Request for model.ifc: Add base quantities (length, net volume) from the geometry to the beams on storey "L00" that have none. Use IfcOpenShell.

First a look at what the model holds.

```python
import ifcopenshell
import ifcopenshell.util.element
import ifcopenshell.util.unit

model = ifcopenshell.open("model.ifc")
print(model.schema)
for unit_type in ("LENGTHUNIT", "AREAUNIT", "VOLUMEUNIT"):
    print(unit_type, ifcopenshell.util.unit.calculate_unit_scale(model, unit_type))
storey = next(s for s in model.by_type("IfcBuildingStorey") if s.Name == "L00")
beams = [e for e in ifcopenshell.util.element.get_decomposition(storey) if e.is_a("IfcBeam")]
for e in sorted(beams, key=lambda e: e.id()):
    print(e.id(), e.is_a(), e.Name, list(ifcopenshell.util.element.get_psets(e, qtos_only=True)), sep=" | ")
```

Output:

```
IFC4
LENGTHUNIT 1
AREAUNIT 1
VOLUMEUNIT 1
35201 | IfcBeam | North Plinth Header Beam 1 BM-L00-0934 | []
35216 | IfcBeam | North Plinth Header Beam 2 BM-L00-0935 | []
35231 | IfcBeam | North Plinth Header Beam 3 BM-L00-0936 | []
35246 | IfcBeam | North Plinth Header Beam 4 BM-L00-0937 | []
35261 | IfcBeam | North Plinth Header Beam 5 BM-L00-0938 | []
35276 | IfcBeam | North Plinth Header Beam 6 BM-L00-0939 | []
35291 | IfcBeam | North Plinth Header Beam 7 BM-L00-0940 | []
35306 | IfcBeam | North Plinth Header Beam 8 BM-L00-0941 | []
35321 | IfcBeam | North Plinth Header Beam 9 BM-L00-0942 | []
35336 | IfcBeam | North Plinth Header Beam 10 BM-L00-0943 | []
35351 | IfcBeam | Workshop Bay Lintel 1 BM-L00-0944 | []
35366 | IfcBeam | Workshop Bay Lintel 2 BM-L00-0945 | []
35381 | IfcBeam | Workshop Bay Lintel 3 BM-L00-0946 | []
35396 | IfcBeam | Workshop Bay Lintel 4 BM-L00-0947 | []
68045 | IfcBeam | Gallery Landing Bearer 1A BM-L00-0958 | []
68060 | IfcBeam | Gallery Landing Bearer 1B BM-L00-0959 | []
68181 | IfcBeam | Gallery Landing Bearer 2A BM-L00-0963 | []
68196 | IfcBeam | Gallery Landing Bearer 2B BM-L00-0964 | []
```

```python
import ifcopenshell
import ifcopenshell.api.pset
import ifcopenshell.geom
import ifcopenshell.util.element
import ifcopenshell.util.shape
import ifcopenshell.util.unit

model = ifcopenshell.open("model.ifc")
unit_scale = ifcopenshell.util.unit.calculate_unit_scale(model)
volume_scale = ifcopenshell.util.unit.calculate_unit_scale(model, "VOLUMEUNIT")
settings = ifcopenshell.geom.settings()

storey = next(s for s in model.by_type("IfcBuildingStorey") if s.Name == "L00")
beams = [e for e in ifcopenshell.util.element.get_decomposition(storey) if e.is_a("IfcBeam")]

for e in sorted(beams, key=lambda e: e.id()):
    if ifcopenshell.util.element.get_psets(e, qtos_only=True, should_inherit=False):
        continue
    # Geometry comes back in metres, in the element's own axes.
    shape = ifcopenshell.geom.create_shape(settings, e)
    values = {
        "Length": ifcopenshell.util.shape.get_max_xyz(shape.geometry) / unit_scale,
        "NetVolume": ifcopenshell.util.shape.get_volume(shape.geometry) / volume_scale,
    }
    qto = ifcopenshell.api.pset.add_qto(model, product=e, name="Qto_BeamBaseQuantities")
    ifcopenshell.api.pset.edit_qto(model, qto=qto, properties=values)
    print(e.id(), {k: round(v, 3) for k, v in values.items()})

model.write("model_rev.ifc")
```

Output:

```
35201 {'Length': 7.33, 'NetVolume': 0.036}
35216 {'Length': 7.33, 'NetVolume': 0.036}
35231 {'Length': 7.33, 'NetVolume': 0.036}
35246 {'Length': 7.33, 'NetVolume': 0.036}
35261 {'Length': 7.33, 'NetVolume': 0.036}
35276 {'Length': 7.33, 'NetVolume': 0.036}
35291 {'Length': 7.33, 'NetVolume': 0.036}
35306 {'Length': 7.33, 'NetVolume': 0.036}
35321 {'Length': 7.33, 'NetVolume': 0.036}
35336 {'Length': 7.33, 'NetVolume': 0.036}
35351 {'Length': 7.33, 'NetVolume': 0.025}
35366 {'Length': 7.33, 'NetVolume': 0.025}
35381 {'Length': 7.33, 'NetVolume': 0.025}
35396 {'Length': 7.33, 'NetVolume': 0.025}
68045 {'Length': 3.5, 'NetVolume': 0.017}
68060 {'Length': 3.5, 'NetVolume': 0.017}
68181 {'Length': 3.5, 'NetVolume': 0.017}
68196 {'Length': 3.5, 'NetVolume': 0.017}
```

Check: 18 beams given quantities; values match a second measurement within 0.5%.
